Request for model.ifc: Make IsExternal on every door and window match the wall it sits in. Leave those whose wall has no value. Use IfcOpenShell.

First a look at what the model holds.

```python
import ifcopenshell
import ifcopenshell.util.element

model = ifcopenshell.open("model.ifc")
print(model.schema)
seen = {}
for e in model.by_type("IfcDoor") + model.by_type("IfcWindow"):
    if not e.FillsVoids:
        continue
    host = e.FillsVoids[0].RelatingOpeningElement.VoidsElements[0].RelatingBuildingElement
    own = ifcopenshell.util.element.get_pset(e, f"Pset_{e.is_a()[3:].removesuffix('StandardCase')}Common", "IsExternal")
    wall = ifcopenshell.util.element.get_pset(host, "Pset_WallCommon", "IsExternal")
    seen[e.is_a(), own, wall] = seen.get((e.is_a(), own, wall), 0) + 1
for (cls, own, wall), count in sorted(seen.items(), key=str):
    print(count, cls, "IsExternal:", own, "| host wall:", wall)
```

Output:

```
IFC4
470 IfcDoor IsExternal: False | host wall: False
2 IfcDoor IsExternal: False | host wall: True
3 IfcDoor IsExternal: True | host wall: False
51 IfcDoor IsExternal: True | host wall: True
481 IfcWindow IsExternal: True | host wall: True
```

```python
import ifcopenshell
import ifcopenshell.api.pset
import ifcopenshell.util.element

model = ifcopenshell.open("model.ifc")

count = 0
for ifc_class, pset_name in (("IfcDoor", "Pset_DoorCommon"), ("IfcWindow", "Pset_WindowCommon")):
    for e in model.by_type(ifc_class):
        if not e.FillsVoids:
            continue
        host = e.FillsVoids[0].RelatingOpeningElement.VoidsElements[0].RelatingBuildingElement
        external = ifcopenshell.util.element.get_pset(host, "Pset_WallCommon", "IsExternal")
        if external is None or ifcopenshell.util.element.get_pset(e, pset_name, "IsExternal") == external:
            continue
        pset = ifcopenshell.api.pset.add_pset(model, product=e, name=pset_name)
        ifcopenshell.api.pset.edit_pset(model, pset=pset, properties={"IsExternal": external})
        count += 1

print(count, "updated")

model.write("model-out.ifc")
```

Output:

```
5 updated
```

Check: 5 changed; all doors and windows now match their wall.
